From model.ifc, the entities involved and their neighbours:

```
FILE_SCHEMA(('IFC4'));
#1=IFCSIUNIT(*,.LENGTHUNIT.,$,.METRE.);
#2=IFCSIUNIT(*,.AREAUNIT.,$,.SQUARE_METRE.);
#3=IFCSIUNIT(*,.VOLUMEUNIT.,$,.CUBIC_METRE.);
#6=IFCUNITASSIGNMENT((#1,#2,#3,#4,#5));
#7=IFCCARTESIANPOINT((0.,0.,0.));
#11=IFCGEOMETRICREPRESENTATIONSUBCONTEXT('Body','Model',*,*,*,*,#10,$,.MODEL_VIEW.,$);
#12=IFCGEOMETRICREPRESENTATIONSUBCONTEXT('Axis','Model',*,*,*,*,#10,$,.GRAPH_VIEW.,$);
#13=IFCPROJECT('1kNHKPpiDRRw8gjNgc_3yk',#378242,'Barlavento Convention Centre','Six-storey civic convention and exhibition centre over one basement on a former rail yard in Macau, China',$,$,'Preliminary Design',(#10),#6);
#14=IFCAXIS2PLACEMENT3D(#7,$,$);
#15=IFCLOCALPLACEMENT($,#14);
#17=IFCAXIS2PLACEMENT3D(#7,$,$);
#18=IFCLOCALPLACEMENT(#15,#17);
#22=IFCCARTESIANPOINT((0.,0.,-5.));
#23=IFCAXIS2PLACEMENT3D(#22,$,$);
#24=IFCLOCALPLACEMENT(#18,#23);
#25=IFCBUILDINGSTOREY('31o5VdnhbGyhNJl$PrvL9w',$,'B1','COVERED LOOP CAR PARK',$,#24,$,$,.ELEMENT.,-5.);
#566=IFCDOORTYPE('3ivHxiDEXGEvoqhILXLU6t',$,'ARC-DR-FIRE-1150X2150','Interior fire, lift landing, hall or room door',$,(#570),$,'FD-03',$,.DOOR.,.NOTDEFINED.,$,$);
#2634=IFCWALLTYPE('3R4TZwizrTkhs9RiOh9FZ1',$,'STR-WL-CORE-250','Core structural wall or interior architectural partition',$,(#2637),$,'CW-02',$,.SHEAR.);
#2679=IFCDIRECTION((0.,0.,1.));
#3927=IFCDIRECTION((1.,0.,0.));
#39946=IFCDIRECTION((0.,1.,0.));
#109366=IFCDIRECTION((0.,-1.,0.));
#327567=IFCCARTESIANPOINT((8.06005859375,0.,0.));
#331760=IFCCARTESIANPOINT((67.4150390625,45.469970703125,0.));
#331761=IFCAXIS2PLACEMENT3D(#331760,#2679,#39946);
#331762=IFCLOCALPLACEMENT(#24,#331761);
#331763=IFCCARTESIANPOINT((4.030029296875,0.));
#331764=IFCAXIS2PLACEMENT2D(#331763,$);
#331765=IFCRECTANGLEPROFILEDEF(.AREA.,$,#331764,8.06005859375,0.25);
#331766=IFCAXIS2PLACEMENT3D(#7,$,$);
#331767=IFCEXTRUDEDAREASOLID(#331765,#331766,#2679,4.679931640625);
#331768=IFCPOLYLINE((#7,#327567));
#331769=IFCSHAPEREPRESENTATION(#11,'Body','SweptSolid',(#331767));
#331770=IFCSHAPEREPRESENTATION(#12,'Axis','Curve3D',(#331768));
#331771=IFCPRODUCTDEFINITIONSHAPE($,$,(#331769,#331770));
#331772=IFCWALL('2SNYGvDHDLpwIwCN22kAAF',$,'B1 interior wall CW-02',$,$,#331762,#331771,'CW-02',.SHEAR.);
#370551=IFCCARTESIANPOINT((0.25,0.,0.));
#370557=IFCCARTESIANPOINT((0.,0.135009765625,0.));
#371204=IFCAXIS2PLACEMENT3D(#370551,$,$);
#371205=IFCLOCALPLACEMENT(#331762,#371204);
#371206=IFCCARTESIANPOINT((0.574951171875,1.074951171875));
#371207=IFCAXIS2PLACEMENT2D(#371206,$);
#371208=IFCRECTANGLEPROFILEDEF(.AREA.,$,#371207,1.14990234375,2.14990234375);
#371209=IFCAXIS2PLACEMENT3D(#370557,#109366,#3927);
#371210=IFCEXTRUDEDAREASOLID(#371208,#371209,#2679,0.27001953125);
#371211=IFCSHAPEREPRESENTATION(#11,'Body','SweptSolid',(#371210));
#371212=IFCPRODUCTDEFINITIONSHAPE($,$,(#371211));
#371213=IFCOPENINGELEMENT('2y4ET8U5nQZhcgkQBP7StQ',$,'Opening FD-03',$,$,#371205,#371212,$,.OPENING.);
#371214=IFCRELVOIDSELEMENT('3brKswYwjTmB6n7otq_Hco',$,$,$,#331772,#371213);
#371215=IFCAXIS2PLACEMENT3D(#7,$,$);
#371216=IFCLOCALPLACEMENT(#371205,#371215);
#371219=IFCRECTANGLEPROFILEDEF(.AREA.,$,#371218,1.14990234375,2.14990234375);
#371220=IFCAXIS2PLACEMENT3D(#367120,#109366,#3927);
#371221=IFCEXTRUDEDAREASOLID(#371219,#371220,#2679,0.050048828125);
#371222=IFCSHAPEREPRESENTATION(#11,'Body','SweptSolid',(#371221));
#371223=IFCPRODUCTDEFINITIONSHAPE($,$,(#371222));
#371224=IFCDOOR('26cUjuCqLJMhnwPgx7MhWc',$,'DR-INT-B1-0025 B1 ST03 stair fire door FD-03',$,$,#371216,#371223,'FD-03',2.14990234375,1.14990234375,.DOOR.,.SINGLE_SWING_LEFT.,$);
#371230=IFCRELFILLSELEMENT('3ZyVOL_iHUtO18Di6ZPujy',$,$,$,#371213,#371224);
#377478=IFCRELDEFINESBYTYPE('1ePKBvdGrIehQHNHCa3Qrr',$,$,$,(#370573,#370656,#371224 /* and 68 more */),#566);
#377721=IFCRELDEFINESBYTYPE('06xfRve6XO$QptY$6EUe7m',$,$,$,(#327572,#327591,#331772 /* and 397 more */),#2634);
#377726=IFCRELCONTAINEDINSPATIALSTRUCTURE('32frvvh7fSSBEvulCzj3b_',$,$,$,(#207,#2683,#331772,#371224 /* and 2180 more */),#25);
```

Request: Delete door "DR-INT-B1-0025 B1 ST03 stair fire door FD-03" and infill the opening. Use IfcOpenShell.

```python
import ifcopenshell
import ifcopenshell.api.feature
import ifcopenshell.api.root
import ifcopenshell.geom
import ifcopenshell.util.shape

model = ifcopenshell.open("model.ifc")
settings = ifcopenshell.geom.settings()


def volume(element):
    """Net volume in cubic metres, openings subtracted."""
    shape = ifcopenshell.geom.create_shape(settings, element)
    return ifcopenshell.util.shape.get_volume(shape.geometry)


door = model.by_id(371224)
opening = door.FillsVoids[0].RelatingOpeningElement
wall = opening.VoidsElements[0].RelatingBuildingElement
before = volume(wall)

ifcopenshell.api.root.remove_product(model, product=door)
ifcopenshell.api.feature.remove_feature(model, feature=opening)

after = volume(wall)

print(f"wall volume {before:.3f} -> {after:.3f} m3")

model.write("model_rev.ifc")
```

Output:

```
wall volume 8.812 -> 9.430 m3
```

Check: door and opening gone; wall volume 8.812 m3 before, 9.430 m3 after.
